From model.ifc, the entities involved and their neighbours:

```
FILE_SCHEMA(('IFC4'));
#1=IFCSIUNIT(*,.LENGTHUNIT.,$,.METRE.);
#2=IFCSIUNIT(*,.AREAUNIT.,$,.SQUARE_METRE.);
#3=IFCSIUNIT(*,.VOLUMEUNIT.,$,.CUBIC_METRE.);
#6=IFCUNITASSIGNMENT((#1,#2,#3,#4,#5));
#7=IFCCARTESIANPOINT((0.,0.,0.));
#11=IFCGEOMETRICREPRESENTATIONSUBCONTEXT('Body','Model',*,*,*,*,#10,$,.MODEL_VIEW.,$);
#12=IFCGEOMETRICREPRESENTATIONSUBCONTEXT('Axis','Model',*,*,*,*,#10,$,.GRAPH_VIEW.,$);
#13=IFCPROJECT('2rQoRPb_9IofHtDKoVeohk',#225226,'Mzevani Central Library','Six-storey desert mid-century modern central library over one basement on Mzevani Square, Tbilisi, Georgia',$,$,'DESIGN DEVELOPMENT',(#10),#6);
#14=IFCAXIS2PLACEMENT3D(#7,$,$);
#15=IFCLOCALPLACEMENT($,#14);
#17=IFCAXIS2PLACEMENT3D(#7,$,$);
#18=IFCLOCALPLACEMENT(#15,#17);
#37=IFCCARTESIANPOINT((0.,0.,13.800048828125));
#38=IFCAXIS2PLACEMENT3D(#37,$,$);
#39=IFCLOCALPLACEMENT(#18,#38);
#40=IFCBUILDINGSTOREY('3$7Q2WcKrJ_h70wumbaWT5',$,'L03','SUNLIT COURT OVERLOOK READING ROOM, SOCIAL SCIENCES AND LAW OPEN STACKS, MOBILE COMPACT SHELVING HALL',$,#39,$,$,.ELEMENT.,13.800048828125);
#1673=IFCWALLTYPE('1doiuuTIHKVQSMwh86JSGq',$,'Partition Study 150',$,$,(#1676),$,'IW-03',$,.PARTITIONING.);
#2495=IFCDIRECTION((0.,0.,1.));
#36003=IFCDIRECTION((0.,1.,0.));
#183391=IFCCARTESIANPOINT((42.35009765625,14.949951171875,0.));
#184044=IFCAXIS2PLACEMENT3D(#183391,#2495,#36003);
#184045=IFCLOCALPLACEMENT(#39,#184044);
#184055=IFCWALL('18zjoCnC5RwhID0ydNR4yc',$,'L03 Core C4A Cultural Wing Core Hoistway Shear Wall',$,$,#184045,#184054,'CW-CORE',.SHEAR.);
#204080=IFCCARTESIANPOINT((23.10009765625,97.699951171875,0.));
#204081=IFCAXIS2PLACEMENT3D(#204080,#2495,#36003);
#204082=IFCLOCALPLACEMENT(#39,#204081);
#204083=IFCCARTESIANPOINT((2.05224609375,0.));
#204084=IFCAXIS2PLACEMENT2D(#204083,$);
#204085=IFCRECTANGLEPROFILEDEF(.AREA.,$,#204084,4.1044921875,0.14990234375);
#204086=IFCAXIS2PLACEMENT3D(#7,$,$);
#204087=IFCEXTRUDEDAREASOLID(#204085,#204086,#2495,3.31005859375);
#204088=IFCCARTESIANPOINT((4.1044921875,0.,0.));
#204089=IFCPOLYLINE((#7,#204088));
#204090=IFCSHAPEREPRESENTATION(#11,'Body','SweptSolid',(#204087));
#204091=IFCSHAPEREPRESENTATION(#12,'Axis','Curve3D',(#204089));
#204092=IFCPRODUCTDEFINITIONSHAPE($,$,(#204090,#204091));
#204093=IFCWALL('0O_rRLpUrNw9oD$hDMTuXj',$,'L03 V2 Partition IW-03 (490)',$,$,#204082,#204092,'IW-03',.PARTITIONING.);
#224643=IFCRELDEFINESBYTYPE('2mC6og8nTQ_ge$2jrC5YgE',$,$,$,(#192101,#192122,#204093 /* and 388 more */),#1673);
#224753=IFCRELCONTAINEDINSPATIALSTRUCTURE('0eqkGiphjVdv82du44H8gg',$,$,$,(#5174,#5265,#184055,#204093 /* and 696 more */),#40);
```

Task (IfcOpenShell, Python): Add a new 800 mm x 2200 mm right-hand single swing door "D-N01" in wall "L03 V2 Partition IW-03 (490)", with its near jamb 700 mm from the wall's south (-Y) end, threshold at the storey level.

```python
import numpy as np
import ifcopenshell
import ifcopenshell.api.feature
import ifcopenshell.api.geometry
import ifcopenshell.api.root
import ifcopenshell.api.spatial
import ifcopenshell.geom
import ifcopenshell.util.element
import ifcopenshell.util.placement
import ifcopenshell.util.representation
import ifcopenshell.util.shape
import ifcopenshell.util.unit

model = ifcopenshell.open("model.ifc")
unit_scale = ifcopenshell.util.unit.calculate_unit_scale(model)
settings = ifcopenshell.geom.settings()


def volume(element):
    """Net volume in cubic metres, openings subtracted."""
    shape = ifcopenshell.geom.create_shape(settings, element)
    return ifcopenshell.util.shape.get_volume(shape.geometry)


wall = model.by_guid("0O_rRLpUrNw9oD$hDMTuXj")
storey = ifcopenshell.util.element.get_container(wall, ifc_class="IfcBuildingStorey")
context = ifcopenshell.util.representation.get_context(model, "Model", "Body", "MODEL_VIEW")
before = volume(wall)

width, height, from_end, sill = 0.8, 2.2, 0.7, 0.0  # metres

# The wall runs along its own X axis, and the end named is its -X end.
wall_shape = ifcopenshell.geom.create_shape(settings, wall)
x, y, z = ifcopenshell.util.shape.get_vertices(wall_shape.geometry).T
start = x.min() + from_end
face, thickness = float(y.min()), float(y.max() - y.min())
wall_matrix = ifcopenshell.util.placement.get_local_placement(wall.ObjectPlacement)
level = ifcopenshell.util.placement.get_local_placement(storey.ObjectPlacement)[2, 3]


def in_wall(x, y):
    """Placement at x, y metres in the wall's axes, at sill height."""
    matrix = wall_matrix.copy()
    matrix[:, 3] = wall_matrix @ np.array([x / unit_scale, y / unit_scale, 0.0, 1.0])
    matrix[2, 3] = level + sill / unit_scale
    return matrix


# Opening: a box that overshoots both wall faces by 50 mm.
opening = ifcopenshell.api.root.create_entity(model, ifc_class="IfcOpeningElement", predefined_type="OPENING")
box = ifcopenshell.api.geometry.add_wall_representation(
    model, context=context, length=width, height=height, thickness=thickness + 0.1
)
ifcopenshell.api.geometry.assign_representation(model, product=opening, representation=box)
ifcopenshell.api.geometry.edit_object_placement(model, product=opening, matrix=in_wall(start, face - 0.05), is_si=False)
ifcopenshell.api.feature.add_feature(model, feature=opening, element=wall)

door = ifcopenshell.api.root.create_entity(model, ifc_class="IfcDoor", name="D-N01", predefined_type="DOOR")
door.OverallWidth, door.OverallHeight = width / unit_scale, height / unit_scale
door.OperationType = "SINGLE_SWING_RIGHT"
body = ifcopenshell.api.geometry.add_door_representation(
    model,
    context=context,
    overall_width=door.OverallWidth,
    overall_height=door.OverallHeight,
    operation_type="SINGLE_SWING_RIGHT",
    lining_properties={"LiningDepth": thickness / unit_scale, "ThresholdDepth": thickness / unit_scale},
)
ifcopenshell.api.geometry.assign_representation(model, product=door, representation=body)
ifcopenshell.api.spatial.assign_container(model, products=[door], relating_structure=storey)
ifcopenshell.api.feature.add_filling(model, opening=opening, element=door)

# The lining spans the wall, so the door starts at the wall face.
ifcopenshell.api.geometry.edit_object_placement(model, product=door, matrix=in_wall(start, face), is_si=False)

after = volume(wall)

print(f"wall volume {before:.3f} -> {after:.3f} m3")

model.write("model_edited.ifc")
```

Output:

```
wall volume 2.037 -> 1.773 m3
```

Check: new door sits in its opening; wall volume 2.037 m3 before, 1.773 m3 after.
